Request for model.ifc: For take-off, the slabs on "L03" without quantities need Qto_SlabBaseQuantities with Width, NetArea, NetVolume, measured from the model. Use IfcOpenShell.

First a look at what the model holds.

```python
import ifcopenshell
import ifcopenshell.util.element
import ifcopenshell.util.unit

model = ifcopenshell.open("model.ifc")
print(model.schema)
for unit_type in ("LENGTHUNIT", "AREAUNIT", "VOLUMEUNIT"):
    print(unit_type, ifcopenshell.util.unit.calculate_unit_scale(model, unit_type))
storey = next(s for s in model.by_type("IfcBuildingStorey") if s.Name == "L03")
slabs = [e for e in ifcopenshell.util.element.get_decomposition(storey) if e.is_a("IfcSlab")]
for e in sorted(slabs, key=lambda e: e.id()):
    print(e.id(), e.is_a(), e.Name, list(ifcopenshell.util.element.get_psets(e, qtos_only=True)), sep=" | ")
```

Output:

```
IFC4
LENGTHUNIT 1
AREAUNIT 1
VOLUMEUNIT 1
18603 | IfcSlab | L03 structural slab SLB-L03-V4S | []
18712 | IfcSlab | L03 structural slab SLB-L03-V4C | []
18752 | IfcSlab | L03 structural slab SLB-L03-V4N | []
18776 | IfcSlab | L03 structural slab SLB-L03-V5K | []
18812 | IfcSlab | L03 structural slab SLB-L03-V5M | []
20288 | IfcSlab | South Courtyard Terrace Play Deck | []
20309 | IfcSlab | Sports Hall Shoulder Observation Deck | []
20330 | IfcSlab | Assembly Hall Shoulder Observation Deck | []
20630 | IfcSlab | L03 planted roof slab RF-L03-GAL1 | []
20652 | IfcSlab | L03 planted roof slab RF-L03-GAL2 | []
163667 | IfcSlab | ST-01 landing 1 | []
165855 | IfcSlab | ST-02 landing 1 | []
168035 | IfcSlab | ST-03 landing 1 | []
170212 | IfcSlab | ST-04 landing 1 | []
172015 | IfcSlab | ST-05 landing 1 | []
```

```python
import ifcopenshell
import ifcopenshell.api.pset
import ifcopenshell.geom
import ifcopenshell.util.element
import ifcopenshell.util.shape
import ifcopenshell.util.unit

model = ifcopenshell.open("model.ifc")
unit_scale = ifcopenshell.util.unit.calculate_unit_scale(model)
area_scale = ifcopenshell.util.unit.calculate_unit_scale(model, "AREAUNIT")
volume_scale = ifcopenshell.util.unit.calculate_unit_scale(model, "VOLUMEUNIT")
settings = ifcopenshell.geom.settings()

storey = next(s for s in model.by_type("IfcBuildingStorey") if s.Name == "L03")
slabs = [e for e in ifcopenshell.util.element.get_decomposition(storey) if e.is_a("IfcSlab")]

for e in sorted(slabs, key=lambda e: e.id()):
    if ifcopenshell.util.element.get_psets(e, qtos_only=True, should_inherit=False):
        continue
    # Geometry comes back in metres, in the element's own axes.
    shape = ifcopenshell.geom.create_shape(settings, e)
    values = {
        "Width": ifcopenshell.util.shape.get_z(shape.geometry) / unit_scale,
        "NetArea": ifcopenshell.util.shape.get_footprint_area(shape.geometry) / area_scale,
        "NetVolume": ifcopenshell.util.shape.get_volume(shape.geometry) / volume_scale,
    }
    qto = ifcopenshell.api.pset.add_qto(model, product=e, name="Qto_SlabBaseQuantities")
    ifcopenshell.api.pset.edit_qto(model, qto=qto, properties=values)
    print(e.id(), {k: round(v, 3) for k, v in values.items()})

model.write("model_rev.ifc")
```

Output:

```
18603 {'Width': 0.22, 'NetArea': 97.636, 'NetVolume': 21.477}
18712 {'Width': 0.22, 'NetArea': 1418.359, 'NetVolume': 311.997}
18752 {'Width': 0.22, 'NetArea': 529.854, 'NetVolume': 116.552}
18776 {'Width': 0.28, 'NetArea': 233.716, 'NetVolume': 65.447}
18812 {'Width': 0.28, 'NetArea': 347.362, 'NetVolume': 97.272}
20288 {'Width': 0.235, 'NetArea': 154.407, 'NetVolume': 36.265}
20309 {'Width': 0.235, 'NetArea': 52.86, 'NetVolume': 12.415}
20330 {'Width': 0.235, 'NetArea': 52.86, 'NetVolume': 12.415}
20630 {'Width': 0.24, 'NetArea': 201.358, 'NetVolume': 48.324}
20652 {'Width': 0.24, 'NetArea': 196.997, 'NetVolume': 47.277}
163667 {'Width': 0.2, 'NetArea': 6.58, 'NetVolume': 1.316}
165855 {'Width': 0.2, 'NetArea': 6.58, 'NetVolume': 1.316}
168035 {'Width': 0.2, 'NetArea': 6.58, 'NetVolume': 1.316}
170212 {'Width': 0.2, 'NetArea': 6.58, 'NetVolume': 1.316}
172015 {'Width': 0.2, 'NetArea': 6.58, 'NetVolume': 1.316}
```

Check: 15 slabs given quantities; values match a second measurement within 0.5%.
